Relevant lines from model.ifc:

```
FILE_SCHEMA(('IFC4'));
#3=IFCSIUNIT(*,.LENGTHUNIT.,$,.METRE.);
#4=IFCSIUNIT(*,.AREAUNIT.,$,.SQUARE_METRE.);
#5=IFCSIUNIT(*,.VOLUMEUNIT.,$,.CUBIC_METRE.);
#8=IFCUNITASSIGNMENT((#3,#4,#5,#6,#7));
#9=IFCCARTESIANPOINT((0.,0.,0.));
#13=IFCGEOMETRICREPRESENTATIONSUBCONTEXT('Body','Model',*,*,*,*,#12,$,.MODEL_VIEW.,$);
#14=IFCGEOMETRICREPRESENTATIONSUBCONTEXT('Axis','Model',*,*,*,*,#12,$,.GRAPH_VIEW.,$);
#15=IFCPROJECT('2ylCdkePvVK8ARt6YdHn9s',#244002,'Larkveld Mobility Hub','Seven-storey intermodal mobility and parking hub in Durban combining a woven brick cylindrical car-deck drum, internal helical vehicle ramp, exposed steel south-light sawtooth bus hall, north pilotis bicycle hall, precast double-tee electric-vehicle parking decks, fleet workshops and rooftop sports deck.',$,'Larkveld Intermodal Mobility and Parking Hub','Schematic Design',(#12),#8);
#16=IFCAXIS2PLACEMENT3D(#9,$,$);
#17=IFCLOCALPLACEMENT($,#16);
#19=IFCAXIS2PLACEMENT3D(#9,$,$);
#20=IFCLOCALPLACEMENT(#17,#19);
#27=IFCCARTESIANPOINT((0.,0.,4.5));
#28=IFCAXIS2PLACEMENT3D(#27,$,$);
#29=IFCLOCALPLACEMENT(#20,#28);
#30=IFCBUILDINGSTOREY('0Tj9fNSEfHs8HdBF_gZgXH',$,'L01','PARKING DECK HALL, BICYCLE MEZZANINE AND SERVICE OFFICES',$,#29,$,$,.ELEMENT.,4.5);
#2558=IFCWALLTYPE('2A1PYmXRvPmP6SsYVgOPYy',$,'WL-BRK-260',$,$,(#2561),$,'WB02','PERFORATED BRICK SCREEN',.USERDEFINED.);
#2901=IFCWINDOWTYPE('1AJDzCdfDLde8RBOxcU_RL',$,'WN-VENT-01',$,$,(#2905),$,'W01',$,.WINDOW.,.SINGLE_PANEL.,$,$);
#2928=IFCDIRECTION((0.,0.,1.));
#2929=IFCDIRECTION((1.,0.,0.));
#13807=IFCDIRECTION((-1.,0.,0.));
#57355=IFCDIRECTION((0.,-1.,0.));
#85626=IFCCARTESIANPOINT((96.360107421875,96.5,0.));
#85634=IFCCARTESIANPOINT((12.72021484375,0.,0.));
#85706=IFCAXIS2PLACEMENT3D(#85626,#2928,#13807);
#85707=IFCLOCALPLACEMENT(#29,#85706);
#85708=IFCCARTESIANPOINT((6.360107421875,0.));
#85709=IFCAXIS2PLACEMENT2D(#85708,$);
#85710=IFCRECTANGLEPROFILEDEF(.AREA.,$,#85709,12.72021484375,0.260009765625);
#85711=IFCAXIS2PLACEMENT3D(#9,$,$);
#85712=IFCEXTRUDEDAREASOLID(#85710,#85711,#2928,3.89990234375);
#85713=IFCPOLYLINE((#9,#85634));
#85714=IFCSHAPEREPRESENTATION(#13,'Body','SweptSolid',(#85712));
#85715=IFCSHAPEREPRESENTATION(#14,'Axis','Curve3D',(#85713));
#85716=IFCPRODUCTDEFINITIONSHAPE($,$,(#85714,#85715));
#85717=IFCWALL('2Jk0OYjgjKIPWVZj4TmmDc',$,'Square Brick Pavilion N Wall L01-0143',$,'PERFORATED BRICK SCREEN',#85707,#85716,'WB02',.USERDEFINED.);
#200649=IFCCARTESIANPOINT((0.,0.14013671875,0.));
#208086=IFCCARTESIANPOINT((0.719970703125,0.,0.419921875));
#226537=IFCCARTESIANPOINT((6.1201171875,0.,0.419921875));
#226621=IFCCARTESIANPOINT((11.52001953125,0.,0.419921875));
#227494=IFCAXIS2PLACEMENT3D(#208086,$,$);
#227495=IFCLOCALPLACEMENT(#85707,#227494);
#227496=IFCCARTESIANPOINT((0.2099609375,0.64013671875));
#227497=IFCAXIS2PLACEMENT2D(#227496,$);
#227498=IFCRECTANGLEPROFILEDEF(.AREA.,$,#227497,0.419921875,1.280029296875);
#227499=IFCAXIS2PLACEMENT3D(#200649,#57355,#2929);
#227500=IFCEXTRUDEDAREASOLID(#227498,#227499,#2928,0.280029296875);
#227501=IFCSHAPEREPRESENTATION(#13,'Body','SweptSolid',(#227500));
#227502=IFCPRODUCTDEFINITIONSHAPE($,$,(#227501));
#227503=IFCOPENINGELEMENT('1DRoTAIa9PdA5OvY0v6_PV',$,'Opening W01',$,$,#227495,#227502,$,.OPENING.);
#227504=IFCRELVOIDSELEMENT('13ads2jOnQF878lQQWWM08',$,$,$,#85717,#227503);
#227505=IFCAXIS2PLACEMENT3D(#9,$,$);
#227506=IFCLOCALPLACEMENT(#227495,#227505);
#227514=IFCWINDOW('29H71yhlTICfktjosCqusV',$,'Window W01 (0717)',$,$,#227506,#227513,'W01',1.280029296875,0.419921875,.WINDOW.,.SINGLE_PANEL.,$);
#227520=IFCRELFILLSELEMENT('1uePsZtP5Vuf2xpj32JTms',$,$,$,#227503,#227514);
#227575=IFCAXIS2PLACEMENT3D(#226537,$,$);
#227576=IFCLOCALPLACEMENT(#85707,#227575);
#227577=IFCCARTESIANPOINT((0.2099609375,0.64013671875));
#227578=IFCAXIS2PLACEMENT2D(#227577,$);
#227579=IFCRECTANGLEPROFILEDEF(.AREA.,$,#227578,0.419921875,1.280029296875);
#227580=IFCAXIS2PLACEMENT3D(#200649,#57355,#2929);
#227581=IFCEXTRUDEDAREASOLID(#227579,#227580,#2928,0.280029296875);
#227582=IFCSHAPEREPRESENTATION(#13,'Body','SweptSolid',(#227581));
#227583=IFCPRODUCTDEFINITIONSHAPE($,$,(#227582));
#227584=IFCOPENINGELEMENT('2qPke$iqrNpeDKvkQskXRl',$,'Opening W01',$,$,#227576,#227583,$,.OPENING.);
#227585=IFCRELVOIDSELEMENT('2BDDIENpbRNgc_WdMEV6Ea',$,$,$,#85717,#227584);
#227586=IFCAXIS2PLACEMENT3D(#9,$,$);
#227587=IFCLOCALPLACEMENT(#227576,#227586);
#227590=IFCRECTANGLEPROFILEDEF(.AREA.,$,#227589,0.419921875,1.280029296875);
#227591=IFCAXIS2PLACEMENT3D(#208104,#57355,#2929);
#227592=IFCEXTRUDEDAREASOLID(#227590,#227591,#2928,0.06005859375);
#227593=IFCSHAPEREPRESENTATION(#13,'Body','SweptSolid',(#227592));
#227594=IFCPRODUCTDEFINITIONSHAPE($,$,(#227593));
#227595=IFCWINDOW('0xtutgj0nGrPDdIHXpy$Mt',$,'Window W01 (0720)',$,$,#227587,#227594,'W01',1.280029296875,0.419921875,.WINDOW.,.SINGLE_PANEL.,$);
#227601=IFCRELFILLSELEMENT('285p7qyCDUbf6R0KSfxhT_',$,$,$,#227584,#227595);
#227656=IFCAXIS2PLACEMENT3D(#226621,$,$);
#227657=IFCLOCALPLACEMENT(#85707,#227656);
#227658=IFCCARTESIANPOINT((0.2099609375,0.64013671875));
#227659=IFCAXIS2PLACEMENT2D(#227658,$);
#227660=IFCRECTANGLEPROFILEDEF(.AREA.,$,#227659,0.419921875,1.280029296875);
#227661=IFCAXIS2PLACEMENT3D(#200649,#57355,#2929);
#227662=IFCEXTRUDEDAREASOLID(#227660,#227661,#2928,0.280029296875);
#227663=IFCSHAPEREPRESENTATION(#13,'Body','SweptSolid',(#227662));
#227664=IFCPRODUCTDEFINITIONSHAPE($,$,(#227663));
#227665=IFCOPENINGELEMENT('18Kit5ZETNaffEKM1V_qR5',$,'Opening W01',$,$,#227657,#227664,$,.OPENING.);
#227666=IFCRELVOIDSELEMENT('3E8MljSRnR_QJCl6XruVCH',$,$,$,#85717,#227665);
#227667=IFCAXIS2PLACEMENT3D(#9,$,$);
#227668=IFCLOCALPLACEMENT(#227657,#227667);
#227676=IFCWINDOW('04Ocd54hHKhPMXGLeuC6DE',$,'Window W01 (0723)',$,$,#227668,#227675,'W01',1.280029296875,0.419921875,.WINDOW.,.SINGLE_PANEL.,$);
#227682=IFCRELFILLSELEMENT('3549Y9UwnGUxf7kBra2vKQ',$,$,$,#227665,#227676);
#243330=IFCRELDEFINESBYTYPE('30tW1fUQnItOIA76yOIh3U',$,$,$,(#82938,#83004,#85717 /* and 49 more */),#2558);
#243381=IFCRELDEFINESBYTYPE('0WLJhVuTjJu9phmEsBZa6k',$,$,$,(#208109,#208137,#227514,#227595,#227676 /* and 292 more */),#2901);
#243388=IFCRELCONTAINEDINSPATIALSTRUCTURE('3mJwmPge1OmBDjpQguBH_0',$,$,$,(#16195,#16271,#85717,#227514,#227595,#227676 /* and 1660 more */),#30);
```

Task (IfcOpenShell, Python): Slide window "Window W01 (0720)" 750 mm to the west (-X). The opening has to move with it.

```python
import ifcopenshell
import ifcopenshell.api.geometry
import ifcopenshell.util.placement

model = ifcopenshell.open("model.ifc")

window = model.by_guid("0xtutgj0nGrPDdIHXpy$Mt")
opening = window.FillsVoids[0].RelatingOpeningElement
wall = opening.VoidsElements[0].RelatingBuildingElement

wall_matrix = ifcopenshell.util.placement.get_local_placement(wall.ObjectPlacement)
shift = wall_matrix[:3, 0] * 0.75
before = ifcopenshell.util.placement.get_local_placement(window.ObjectPlacement)[:3, 3].copy()

# The window is placed relative to its opening, so it follows when the opening moves.
matrix = ifcopenshell.util.placement.get_local_placement(opening.ObjectPlacement)
matrix[:3, 3] += shift
ifcopenshell.api.geometry.edit_object_placement(
    model, product=opening, matrix=matrix, is_si=False, should_transform_children=True
)

after = ifcopenshell.util.placement.get_local_placement(window.ObjectPlacement)[:3, 3]
print("window moved by", (after - before).round(3) + 0.0)

model.write("model_v2.ifc")
```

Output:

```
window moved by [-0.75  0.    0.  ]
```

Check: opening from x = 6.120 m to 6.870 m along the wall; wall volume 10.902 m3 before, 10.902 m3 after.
